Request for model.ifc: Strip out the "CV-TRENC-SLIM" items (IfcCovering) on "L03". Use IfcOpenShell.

First a look at what the model holds.

```python
import ifcopenshell
import ifcopenshell.util.element

model = ifcopenshell.open("model.ifc")
print(model.schema)
storey = next(s for s in model.by_type("IfcBuildingStorey") if s.Name == "L03")
coverings = [e for e in ifcopenshell.util.element.get_decomposition(storey) if e.is_a("IfcCovering")]
seen = {}
for e in coverings:
    element_type = ifcopenshell.util.element.get_type(e)
    name = element_type.Name if element_type not in (None, e) else None
    seen[name] = seen.get(name, 0) + 1
for name, count in sorted(seen.items(), key=str):
    print(count, "x", name)
```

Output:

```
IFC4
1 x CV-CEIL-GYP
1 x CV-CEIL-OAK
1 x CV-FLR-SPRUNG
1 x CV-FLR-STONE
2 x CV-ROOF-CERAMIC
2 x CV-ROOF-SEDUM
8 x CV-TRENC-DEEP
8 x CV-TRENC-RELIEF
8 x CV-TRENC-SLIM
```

```python
import ifcopenshell
import ifcopenshell.api.root
import ifcopenshell.util.element

model = ifcopenshell.open("model.ifc")

storey = next(s for s in model.by_type("IfcBuildingStorey") if s.Name == "L03")
coverings = [e for e in ifcopenshell.util.element.get_decomposition(storey) if e.is_a("IfcCovering")]
targets = [e for e in coverings if (t := ifcopenshell.util.element.get_type(e)) not in (None, e) and t.Name == "CV-TRENC-SLIM"]

for e in targets:
    ifcopenshell.api.root.remove_product(model, product=e)
print(len(targets), "removed")

model.write("model-out.ifc")
```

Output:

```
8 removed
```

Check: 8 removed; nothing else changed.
